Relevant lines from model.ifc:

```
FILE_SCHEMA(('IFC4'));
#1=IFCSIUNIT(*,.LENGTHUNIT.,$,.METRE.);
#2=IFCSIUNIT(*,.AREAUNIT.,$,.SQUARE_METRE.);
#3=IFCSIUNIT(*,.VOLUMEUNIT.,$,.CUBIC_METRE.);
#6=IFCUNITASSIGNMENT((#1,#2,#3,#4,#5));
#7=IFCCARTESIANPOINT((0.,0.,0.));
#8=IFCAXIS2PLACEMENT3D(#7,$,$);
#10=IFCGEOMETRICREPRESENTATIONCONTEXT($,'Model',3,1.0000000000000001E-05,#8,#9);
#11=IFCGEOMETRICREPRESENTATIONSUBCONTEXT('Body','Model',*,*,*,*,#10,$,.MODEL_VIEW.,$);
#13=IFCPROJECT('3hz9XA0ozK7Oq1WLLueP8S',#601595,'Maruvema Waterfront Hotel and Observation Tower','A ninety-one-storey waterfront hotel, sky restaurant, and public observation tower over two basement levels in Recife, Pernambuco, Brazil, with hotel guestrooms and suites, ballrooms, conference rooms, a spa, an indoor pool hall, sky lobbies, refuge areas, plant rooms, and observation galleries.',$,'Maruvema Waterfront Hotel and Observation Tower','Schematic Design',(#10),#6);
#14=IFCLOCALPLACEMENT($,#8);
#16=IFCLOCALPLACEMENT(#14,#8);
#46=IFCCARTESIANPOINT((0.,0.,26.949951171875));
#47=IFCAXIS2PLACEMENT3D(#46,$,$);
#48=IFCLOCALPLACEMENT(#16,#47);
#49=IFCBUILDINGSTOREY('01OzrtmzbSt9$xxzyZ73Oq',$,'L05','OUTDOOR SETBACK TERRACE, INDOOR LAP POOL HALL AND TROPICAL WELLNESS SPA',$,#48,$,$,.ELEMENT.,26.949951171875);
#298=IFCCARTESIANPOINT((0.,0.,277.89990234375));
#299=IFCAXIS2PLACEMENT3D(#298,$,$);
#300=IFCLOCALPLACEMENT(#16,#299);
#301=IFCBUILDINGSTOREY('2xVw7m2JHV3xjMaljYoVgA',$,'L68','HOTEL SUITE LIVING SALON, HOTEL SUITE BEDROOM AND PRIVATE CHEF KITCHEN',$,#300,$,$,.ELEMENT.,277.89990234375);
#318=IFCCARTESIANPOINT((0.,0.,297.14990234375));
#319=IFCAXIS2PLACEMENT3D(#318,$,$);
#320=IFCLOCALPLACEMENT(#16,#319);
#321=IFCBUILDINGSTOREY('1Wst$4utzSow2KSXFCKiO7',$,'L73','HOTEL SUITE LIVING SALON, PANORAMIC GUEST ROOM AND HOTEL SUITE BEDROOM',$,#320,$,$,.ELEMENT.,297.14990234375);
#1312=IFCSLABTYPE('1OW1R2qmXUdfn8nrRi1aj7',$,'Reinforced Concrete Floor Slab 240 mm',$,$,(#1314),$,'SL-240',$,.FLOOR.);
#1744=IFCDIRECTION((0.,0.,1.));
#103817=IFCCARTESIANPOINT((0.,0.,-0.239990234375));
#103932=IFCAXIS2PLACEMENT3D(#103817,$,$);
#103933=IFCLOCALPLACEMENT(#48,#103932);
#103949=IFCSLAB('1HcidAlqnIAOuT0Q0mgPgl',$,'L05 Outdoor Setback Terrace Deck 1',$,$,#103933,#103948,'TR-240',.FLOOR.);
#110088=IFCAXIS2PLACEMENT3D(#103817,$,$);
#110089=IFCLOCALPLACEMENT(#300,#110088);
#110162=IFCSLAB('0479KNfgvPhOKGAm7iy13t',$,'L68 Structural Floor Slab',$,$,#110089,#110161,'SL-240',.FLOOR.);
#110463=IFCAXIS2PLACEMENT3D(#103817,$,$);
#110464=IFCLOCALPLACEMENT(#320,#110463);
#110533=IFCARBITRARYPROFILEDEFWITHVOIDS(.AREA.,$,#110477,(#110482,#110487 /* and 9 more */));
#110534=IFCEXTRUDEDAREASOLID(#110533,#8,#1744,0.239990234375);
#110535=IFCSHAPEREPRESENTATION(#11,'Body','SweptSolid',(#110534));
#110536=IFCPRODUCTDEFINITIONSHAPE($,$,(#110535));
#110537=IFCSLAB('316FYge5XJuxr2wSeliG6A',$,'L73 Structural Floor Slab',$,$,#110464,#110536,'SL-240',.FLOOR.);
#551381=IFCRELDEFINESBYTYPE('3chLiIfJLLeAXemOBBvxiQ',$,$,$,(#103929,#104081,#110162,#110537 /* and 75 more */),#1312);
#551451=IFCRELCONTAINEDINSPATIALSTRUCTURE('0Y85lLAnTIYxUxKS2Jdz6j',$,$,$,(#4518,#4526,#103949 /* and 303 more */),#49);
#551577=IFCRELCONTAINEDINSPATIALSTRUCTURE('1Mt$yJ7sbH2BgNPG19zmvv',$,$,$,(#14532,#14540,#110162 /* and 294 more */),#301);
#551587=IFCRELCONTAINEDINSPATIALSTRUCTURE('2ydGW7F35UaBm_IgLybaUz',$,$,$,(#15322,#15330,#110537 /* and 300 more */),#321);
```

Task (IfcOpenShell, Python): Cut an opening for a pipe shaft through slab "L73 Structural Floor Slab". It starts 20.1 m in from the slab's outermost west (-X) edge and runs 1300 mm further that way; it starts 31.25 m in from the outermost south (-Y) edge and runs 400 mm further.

```python
import numpy as np
import ifcopenshell
import ifcopenshell.api.feature
import ifcopenshell.api.geometry
import ifcopenshell.api.root
import ifcopenshell.geom
import ifcopenshell.util.placement
import ifcopenshell.util.representation
import ifcopenshell.util.shape
import ifcopenshell.util.unit

model = ifcopenshell.open("model.ifc")
unit_scale = ifcopenshell.util.unit.calculate_unit_scale(model)
settings = ifcopenshell.geom.settings()


def volume(element):
    """Net volume in cubic metres, openings subtracted."""
    shape = ifcopenshell.geom.create_shape(settings, element)
    return ifcopenshell.util.shape.get_volume(shape.geometry)


slab = model.by_guid("316FYge5XJuxr2wSeliG6A")
before = volume(slab)

# Extent in the slab's own axes, in metres. The edges named are its -X and -Y sides.
slab_shape = ifcopenshell.geom.create_shape(settings, slab)
vertices = ifcopenshell.util.shape.get_vertices(slab_shape.geometry)
x_min, y_min, bottom = vertices.min(axis=0)
top = vertices[:, 2].max()

opening = ifcopenshell.api.root.create_entity(model, ifc_class="IfcOpeningElement", name="Pipe shaft opening", predefined_type="OPENING")
context = ifcopenshell.util.representation.get_context(model, "Model", "Body", "MODEL_VIEW")
width, depth = 1.3, 0.4
outline = [(0.0, 0.0), (width, 0.0), (width, depth), (0.0, depth), (0.0, 0.0)]
# Overshoot both faces by 50 mm so the cut is clean.
shape = ifcopenshell.api.geometry.add_slab_representation(
    model, context=context, depth=top - bottom + 0.1, polyline=outline
)
ifcopenshell.api.geometry.assign_representation(model, product=opening, representation=shape)

matrix = ifcopenshell.util.placement.get_local_placement(slab.ObjectPlacement)
matrix[:, 3] = matrix @ np.append(np.array([x_min + 20.1, y_min + 31.25, bottom - 0.05]) / unit_scale, 1.0)
ifcopenshell.api.geometry.edit_object_placement(model, product=opening, matrix=matrix, is_si=False)
ifcopenshell.api.feature.add_feature(model, feature=opening, element=slab)

after = volume(slab)

print(f"slab volume {before:.3f} -> {after:.3f} m3")

model.write("model_updated.ifc")
```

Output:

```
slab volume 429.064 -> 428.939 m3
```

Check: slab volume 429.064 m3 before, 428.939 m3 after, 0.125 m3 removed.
